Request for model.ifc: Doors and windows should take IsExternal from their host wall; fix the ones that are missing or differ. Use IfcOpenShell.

First a look at what the model holds.

```python
import ifcopenshell
import ifcopenshell.util.element

model = ifcopenshell.open("model.ifc")
print(model.schema)
seen = {}
for e in model.by_type("IfcDoor") + model.by_type("IfcWindow"):
    if not e.FillsVoids:
        continue
    host = e.FillsVoids[0].RelatingOpeningElement.VoidsElements[0].RelatingBuildingElement
    own = ifcopenshell.util.element.get_pset(e, f"Pset_{e.is_a()[3:].removesuffix('StandardCase')}Common", "IsExternal")
    wall = ifcopenshell.util.element.get_pset(host, "Pset_WallCommon", "IsExternal")
    seen[e.is_a(), own, wall] = seen.get((e.is_a(), own, wall), 0) + 1
for (cls, own, wall), count in sorted(seen.items(), key=str):
    print(count, cls, "IsExternal:", own, "| host wall:", wall)
```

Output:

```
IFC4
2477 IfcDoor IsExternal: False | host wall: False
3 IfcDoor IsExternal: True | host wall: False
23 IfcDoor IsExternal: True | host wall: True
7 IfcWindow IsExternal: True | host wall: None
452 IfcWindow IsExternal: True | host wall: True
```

```python
import ifcopenshell
import ifcopenshell.api.pset
import ifcopenshell.util.element

model = ifcopenshell.open("model.ifc")

count = 0
for ifc_class, pset_name in (("IfcDoor", "Pset_DoorCommon"), ("IfcWindow", "Pset_WindowCommon")):
    for e in model.by_type(ifc_class):
        if not e.FillsVoids:
            continue
        host = e.FillsVoids[0].RelatingOpeningElement.VoidsElements[0].RelatingBuildingElement
        external = ifcopenshell.util.element.get_pset(host, "Pset_WallCommon", "IsExternal")
        if external is None or ifcopenshell.util.element.get_pset(e, pset_name, "IsExternal") == external:
            continue
        pset = ifcopenshell.api.pset.add_pset(model, product=e, name=pset_name)
        ifcopenshell.api.pset.edit_pset(model, pset=pset, properties={"IsExternal": external})
        count += 1

print(count, "updated")

model.write("model_updated.ifc")
```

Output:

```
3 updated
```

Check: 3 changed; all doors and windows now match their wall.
